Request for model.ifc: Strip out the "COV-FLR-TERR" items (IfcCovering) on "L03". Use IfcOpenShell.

First a look at what the model holds.

```python
import ifcopenshell
import ifcopenshell.util.element

model = ifcopenshell.open("model.ifc")
print(model.schema)
storey = next(s for s in model.by_type("IfcBuildingStorey") if s.Name == "L03")
coverings = [e for e in ifcopenshell.util.element.get_decomposition(storey) if e.is_a("IfcCovering")]
seen = {}
for e in coverings:
    element_type = ifcopenshell.util.element.get_type(e)
    name = element_type.Name if element_type not in (None, e) else None
    seen[name] = seen.get(name, 0) + 1
for name, count in sorted(seen.items(), key=str):
    print(count, "x", name)
```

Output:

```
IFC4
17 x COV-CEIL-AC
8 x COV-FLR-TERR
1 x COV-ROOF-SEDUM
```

```python
import ifcopenshell
import ifcopenshell.api.root
import ifcopenshell.util.element

model = ifcopenshell.open("model.ifc")

storey = next(s for s in model.by_type("IfcBuildingStorey") if s.Name == "L03")
coverings = [e for e in ifcopenshell.util.element.get_decomposition(storey) if e.is_a("IfcCovering")]
targets = [e for e in coverings if (t := ifcopenshell.util.element.get_type(e)) not in (None, e) and t.Name == "COV-FLR-TERR"]

for e in targets:
    ifcopenshell.api.root.remove_product(model, product=e)
print(len(targets), "removed")

model.write("model_rev.ifc")
```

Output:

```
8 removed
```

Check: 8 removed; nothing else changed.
